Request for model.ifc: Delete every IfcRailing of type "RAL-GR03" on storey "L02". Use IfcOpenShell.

First a look at what the model holds.

```python
import ifcopenshell
import ifcopenshell.util.element

model = ifcopenshell.open("model.ifc")
print(model.schema)
storey = next(s for s in model.by_type("IfcBuildingStorey") if s.Name == "L02")
railings = [e for e in ifcopenshell.util.element.get_decomposition(storey) if e.is_a("IfcRailing")]
seen = {}
for e in railings:
    element_type = ifcopenshell.util.element.get_type(e)
    name = element_type.Name if element_type not in (None, e) else None
    seen[name] = seen.get(name, 0) + 1
for name, count in sorted(seen.items(), key=str):
    print(count, "x", name)
```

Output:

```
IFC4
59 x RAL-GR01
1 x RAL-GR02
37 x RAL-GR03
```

```python
import ifcopenshell
import ifcopenshell.api.root
import ifcopenshell.util.element

model = ifcopenshell.open("model.ifc")

storey = next(s for s in model.by_type("IfcBuildingStorey") if s.Name == "L02")
railings = [e for e in ifcopenshell.util.element.get_decomposition(storey) if e.is_a("IfcRailing")]
targets = [e for e in railings if (t := ifcopenshell.util.element.get_type(e)) not in (None, e) and t.Name == "RAL-GR03"]

for e in targets:
    ifcopenshell.api.root.remove_product(model, product=e)
print(len(targets), "removed")

model.write("model_rev.ifc")
```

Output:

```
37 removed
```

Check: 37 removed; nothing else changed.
